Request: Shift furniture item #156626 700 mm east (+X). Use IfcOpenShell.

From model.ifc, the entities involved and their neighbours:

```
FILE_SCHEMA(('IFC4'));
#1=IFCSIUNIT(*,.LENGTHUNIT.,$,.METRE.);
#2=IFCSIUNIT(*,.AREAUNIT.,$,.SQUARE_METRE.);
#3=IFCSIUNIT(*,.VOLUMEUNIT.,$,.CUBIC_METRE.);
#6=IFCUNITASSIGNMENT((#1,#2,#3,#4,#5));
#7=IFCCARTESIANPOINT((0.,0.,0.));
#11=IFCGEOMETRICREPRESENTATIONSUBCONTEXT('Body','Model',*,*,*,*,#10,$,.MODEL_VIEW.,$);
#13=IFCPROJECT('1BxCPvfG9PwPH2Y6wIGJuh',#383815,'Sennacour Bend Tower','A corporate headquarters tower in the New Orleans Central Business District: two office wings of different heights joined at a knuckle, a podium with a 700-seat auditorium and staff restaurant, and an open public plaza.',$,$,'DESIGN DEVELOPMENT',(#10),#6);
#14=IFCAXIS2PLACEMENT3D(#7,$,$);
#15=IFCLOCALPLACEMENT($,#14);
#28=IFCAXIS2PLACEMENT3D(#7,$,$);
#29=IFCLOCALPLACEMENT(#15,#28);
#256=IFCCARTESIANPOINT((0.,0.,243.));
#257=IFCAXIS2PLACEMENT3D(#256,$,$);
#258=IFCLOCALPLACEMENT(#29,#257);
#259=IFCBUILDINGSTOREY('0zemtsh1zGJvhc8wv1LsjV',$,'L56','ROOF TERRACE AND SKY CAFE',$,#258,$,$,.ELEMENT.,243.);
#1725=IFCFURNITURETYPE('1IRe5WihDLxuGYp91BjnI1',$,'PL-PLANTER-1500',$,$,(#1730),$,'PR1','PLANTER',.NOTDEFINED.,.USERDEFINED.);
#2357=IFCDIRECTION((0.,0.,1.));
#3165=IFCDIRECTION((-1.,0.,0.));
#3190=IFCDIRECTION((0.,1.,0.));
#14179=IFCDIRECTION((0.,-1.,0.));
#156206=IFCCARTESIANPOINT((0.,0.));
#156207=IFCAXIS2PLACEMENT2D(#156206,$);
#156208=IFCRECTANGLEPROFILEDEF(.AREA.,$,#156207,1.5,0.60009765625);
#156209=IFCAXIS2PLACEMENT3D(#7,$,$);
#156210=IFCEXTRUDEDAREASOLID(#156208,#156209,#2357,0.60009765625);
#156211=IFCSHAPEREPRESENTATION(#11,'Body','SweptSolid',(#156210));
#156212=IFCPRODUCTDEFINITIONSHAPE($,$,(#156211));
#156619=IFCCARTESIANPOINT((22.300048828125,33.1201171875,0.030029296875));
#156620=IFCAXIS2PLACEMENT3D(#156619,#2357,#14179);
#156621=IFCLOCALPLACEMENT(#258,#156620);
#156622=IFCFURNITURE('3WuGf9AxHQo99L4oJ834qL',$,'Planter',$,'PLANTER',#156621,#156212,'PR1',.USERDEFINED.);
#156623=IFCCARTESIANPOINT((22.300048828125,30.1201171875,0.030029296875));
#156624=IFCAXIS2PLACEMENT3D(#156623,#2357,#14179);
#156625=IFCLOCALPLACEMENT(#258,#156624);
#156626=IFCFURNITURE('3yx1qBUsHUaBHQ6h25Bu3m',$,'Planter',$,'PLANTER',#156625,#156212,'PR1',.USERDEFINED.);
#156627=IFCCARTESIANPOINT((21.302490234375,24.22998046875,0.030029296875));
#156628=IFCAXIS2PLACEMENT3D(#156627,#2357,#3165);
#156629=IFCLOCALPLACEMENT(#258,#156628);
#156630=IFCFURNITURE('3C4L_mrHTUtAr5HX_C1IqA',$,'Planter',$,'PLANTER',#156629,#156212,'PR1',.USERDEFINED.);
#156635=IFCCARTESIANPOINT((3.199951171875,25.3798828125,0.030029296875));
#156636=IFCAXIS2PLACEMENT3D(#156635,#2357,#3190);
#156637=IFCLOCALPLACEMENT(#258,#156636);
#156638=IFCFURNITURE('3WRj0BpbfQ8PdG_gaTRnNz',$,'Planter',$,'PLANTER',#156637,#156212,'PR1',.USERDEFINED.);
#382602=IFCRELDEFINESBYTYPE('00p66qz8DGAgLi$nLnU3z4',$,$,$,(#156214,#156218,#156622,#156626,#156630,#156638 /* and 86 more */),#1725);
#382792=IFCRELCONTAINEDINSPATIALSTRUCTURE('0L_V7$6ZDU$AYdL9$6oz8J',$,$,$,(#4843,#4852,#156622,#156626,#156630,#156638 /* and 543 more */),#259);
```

```python
import ifcopenshell
import ifcopenshell.api.geometry
import ifcopenshell.util.placement

model = ifcopenshell.open("model.ifc")

item = model.by_guid("3yx1qBUsHUaBHQ6h25Bu3m")
matrix = ifcopenshell.util.placement.get_local_placement(item.ObjectPlacement)
matrix[0, 3] += 0.7
ifcopenshell.api.geometry.edit_object_placement(model, product=item, matrix=matrix, is_si=False)

print(ifcopenshell.util.placement.get_local_placement(item.ObjectPlacement).round(3) + 0.0)

model.write("model_updated.ifc")
```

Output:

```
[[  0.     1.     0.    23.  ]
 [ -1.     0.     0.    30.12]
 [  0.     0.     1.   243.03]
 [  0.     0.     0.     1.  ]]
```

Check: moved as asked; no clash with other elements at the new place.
